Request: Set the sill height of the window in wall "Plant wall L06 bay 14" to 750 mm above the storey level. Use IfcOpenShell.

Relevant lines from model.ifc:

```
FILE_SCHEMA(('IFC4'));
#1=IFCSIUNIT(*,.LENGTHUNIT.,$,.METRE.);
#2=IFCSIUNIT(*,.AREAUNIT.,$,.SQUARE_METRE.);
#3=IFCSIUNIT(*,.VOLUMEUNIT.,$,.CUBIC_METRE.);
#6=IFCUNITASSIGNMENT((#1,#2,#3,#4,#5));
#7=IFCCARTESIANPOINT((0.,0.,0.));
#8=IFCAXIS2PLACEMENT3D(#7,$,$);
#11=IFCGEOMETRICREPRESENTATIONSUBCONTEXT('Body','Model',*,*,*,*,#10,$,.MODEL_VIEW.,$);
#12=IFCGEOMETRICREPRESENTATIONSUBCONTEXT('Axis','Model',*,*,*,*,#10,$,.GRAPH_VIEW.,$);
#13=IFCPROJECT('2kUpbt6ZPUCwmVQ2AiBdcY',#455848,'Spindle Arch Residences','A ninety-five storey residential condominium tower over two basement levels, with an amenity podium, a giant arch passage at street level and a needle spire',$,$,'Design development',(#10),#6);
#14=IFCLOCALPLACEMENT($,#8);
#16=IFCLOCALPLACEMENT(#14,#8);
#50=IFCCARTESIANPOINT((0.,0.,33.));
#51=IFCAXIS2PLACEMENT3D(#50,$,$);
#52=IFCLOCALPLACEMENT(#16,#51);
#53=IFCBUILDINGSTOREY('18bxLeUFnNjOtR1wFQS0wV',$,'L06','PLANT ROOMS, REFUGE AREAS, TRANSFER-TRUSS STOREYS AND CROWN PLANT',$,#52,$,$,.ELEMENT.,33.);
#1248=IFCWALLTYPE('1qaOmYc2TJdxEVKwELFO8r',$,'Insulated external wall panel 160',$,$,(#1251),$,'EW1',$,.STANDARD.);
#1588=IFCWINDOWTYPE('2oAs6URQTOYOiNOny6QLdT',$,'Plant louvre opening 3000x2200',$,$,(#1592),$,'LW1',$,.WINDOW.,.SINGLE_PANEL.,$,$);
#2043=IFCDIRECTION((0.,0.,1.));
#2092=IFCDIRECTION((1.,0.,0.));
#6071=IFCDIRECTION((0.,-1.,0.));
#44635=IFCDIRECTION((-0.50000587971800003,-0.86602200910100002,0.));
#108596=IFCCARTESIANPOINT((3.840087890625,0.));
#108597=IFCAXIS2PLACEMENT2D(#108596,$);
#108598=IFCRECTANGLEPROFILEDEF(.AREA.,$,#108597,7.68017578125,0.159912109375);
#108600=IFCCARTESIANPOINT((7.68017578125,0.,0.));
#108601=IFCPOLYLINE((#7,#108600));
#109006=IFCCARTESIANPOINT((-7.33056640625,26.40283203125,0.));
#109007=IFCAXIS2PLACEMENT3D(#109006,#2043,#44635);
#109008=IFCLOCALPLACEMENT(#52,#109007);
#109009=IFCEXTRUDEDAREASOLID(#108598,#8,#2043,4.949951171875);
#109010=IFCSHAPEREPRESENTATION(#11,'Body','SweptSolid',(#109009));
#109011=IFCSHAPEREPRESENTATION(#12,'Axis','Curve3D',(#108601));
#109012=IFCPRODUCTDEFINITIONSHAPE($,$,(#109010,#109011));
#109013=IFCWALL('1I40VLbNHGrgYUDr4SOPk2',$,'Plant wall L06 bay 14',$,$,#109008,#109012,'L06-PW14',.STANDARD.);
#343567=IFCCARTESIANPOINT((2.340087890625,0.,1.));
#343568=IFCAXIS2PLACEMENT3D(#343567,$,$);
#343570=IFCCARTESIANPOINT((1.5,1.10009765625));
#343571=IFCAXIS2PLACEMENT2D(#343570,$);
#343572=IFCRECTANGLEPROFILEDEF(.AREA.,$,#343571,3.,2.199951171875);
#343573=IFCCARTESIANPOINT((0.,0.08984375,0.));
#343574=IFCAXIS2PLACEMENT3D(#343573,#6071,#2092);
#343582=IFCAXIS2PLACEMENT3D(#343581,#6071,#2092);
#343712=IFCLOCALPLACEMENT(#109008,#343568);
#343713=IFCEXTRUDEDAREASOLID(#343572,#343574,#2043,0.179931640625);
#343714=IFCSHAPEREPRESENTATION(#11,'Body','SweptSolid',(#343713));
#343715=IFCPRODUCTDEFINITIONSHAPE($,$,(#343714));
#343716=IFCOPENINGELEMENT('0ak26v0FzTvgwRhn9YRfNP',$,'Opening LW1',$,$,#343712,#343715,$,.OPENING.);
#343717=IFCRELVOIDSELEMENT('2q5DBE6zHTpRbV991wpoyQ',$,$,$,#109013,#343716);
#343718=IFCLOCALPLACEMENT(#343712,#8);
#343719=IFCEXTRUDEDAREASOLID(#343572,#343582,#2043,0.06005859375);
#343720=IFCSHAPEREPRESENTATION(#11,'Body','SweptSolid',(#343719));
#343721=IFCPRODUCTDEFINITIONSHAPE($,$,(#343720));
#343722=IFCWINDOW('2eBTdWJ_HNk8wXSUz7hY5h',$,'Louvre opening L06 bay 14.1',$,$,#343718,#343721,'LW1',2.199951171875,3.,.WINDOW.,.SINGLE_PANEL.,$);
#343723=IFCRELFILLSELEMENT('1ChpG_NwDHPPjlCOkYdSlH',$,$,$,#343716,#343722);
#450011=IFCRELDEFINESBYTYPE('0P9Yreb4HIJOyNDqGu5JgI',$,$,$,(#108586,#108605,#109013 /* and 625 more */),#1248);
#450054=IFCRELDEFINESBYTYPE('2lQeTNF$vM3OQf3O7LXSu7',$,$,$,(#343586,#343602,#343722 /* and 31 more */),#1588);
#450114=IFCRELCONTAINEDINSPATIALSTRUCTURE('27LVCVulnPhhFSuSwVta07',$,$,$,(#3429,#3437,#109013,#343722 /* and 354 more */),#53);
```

```python
import numpy as np
import ifcopenshell
import ifcopenshell.api.geometry
import ifcopenshell.geom
import ifcopenshell.util.element
import ifcopenshell.util.placement
import ifcopenshell.util.shape
import ifcopenshell.util.unit

model = ifcopenshell.open("model.ifc")
unit_scale = ifcopenshell.util.unit.calculate_unit_scale(model)

window = model.by_guid("2eBTdWJ_HNk8wXSUz7hY5h")
opening = window.FillsVoids[0].RelatingOpeningElement
storey = ifcopenshell.util.element.get_container(window, ifc_class="IfcBuildingStorey")
level = ifcopenshell.util.placement.get_local_placement(storey.ObjectPlacement)[2, 3]

# The opening's origin need not be at the sill, so measure its lowest point.
shape = ifcopenshell.geom.create_shape(ifcopenshell.geom.settings(), opening)
bottom = ifcopenshell.util.shape.get_shape_bottom_elevation(shape, shape.geometry) / unit_scale
dz = level + 0.75 / unit_scale - bottom

shift = np.array([0.0, 0.0, dz])
# The window is placed relative to its opening, so it follows when the opening moves.
matrix = ifcopenshell.util.placement.get_local_placement(opening.ObjectPlacement)
matrix[:3, 3] += shift
ifcopenshell.api.geometry.edit_object_placement(
    model, product=opening, matrix=matrix, is_si=False, should_transform_children=True
)

print(f"moved by {dz * unit_scale:+.3f} m")

model.write("model-out.ifc")
```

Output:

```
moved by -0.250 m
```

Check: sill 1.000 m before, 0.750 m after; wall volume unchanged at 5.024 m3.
